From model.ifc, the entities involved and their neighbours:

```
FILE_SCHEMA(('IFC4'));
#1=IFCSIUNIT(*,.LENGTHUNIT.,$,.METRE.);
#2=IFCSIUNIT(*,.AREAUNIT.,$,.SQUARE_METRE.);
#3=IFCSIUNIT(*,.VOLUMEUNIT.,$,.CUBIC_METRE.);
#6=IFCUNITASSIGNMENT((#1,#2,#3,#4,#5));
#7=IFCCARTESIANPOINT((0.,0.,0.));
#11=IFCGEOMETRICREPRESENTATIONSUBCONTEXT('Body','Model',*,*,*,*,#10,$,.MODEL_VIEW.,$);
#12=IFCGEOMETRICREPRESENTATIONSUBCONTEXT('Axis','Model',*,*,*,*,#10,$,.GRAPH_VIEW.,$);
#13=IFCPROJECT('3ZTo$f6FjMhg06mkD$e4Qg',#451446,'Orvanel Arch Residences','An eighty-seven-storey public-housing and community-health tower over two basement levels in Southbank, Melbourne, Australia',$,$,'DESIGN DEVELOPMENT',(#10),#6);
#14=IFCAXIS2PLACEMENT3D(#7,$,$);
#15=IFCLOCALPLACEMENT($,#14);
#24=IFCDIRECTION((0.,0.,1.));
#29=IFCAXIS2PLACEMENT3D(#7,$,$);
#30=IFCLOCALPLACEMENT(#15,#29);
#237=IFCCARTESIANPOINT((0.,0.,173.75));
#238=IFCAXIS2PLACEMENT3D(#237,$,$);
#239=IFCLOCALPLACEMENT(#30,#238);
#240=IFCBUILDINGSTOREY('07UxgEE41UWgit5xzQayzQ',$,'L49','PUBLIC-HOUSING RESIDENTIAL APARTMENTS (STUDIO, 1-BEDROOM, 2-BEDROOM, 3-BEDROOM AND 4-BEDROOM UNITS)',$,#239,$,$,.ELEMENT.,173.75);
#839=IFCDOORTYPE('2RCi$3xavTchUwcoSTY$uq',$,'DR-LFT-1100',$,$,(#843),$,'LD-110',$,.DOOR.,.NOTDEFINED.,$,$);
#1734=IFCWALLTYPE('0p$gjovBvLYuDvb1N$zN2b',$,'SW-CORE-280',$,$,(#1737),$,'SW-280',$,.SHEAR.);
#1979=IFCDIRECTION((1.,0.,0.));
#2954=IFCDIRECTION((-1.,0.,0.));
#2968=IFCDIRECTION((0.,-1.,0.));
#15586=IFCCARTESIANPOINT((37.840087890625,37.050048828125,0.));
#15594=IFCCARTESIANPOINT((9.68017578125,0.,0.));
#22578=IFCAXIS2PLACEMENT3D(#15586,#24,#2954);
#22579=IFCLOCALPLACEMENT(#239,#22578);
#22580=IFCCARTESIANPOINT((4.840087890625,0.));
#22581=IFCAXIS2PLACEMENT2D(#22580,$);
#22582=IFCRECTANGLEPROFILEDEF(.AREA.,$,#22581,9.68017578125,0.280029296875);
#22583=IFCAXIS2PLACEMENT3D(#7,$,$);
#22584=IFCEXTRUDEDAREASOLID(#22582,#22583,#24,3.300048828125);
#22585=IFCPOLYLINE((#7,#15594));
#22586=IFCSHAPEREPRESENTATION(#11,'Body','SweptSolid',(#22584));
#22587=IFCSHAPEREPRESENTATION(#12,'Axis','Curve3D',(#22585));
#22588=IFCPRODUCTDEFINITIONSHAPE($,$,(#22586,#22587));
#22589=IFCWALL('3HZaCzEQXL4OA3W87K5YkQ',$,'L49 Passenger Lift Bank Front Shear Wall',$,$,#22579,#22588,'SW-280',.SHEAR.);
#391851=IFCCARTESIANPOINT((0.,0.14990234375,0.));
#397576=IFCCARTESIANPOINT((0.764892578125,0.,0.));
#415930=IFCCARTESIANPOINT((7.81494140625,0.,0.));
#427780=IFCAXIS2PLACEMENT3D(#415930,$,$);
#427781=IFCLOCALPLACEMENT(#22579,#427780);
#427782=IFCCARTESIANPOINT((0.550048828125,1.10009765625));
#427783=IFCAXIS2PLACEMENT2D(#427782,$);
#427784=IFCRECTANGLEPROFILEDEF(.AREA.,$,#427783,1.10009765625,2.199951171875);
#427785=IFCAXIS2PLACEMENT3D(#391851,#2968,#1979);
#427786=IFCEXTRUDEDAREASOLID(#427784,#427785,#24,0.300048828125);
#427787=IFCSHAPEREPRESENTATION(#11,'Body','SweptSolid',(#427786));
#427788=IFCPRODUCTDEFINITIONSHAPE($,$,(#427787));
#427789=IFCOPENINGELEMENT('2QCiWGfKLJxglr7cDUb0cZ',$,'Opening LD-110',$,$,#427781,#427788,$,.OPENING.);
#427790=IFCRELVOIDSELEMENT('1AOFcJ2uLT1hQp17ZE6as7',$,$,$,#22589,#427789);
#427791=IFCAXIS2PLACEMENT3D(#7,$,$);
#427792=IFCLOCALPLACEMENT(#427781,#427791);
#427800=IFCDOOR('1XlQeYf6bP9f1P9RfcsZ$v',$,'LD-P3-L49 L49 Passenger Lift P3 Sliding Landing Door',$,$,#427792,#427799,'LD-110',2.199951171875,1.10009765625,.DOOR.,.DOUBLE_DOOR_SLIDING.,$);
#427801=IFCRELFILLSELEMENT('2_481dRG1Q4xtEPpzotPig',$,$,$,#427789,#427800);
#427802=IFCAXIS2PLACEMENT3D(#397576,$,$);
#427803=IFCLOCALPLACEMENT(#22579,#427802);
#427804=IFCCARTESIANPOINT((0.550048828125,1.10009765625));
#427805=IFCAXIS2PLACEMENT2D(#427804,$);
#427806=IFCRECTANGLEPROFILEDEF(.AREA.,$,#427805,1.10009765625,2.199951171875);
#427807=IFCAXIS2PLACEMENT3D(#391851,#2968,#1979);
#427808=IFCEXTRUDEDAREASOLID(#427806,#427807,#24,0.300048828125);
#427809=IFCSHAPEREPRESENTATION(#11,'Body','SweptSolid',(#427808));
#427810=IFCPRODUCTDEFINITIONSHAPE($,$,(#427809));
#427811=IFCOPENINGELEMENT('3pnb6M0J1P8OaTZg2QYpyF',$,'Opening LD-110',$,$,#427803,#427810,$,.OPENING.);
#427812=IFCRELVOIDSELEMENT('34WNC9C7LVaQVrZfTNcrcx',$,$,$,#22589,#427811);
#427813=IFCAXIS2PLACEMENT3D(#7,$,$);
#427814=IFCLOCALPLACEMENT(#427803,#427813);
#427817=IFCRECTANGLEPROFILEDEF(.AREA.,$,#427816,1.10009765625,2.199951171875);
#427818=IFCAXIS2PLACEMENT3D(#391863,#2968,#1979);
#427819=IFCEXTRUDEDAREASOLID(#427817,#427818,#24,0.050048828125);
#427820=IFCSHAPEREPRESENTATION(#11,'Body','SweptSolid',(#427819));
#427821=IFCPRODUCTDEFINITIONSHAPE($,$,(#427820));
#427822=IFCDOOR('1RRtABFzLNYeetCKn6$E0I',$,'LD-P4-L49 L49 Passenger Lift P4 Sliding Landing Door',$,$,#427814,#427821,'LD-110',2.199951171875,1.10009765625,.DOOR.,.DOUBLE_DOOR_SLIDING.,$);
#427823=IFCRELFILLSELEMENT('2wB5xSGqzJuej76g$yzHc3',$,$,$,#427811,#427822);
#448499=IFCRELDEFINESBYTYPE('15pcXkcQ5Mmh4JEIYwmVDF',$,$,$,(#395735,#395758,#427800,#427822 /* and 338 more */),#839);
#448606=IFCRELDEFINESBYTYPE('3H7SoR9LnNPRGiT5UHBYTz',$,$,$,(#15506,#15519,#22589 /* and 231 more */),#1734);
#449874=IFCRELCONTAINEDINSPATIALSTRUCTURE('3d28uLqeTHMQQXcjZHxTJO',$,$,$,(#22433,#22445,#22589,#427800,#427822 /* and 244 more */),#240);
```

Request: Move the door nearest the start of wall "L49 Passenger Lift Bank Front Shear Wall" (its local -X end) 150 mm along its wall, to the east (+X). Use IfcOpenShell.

```python
import ifcopenshell
import ifcopenshell.api.geometry
import ifcopenshell.util.placement
import ifcopenshell.util.unit

model = ifcopenshell.open("model.ifc")
unit_scale = ifcopenshell.util.unit.calculate_unit_scale(model)

door = model.by_guid("1RRtABFzLNYeetCKn6$E0I")
opening = door.FillsVoids[0].RelatingOpeningElement
wall = opening.VoidsElements[0].RelatingBuildingElement

wall_matrix = ifcopenshell.util.placement.get_local_placement(wall.ObjectPlacement)
shift = wall_matrix[:3, 0] * -0.15 / unit_scale
before = ifcopenshell.util.placement.get_local_placement(door.ObjectPlacement)[:3, 3].copy()

# The door is placed relative to its opening, so it follows when the opening moves.
matrix = ifcopenshell.util.placement.get_local_placement(opening.ObjectPlacement)
matrix[:3, 3] += shift
ifcopenshell.api.geometry.edit_object_placement(
    model, product=opening, matrix=matrix, is_si=False, should_transform_children=True
)

after = ifcopenshell.util.placement.get_local_placement(door.ObjectPlacement)[:3, 3]
print("door moved by", (after - before).round(3) + 0.0)

model.write("model-out.ifc")
```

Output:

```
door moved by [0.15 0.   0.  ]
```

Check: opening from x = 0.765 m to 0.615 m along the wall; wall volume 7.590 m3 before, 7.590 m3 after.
